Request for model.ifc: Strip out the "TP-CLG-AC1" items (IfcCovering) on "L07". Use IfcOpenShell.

First a look at what the model holds.

```python
import ifcopenshell
import ifcopenshell.util.element

model = ifcopenshell.open("model.ifc")
print(model.schema)
storey = next(s for s in model.by_type("IfcBuildingStorey") if s.Name == "L07")
coverings = [e for e in ifcopenshell.util.element.get_decomposition(storey) if e.is_a("IfcCovering")]
seen = {}
for e in coverings:
    element_type = ifcopenshell.util.element.get_type(e)
    name = element_type.Name if element_type not in (None, e) else None
    seen[name] = seen.get(name, 0) + 1
for name, count in sorted(seen.items(), key=str):
    print(count, "x", name)
```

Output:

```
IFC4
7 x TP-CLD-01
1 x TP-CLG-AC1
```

```python
import ifcopenshell
import ifcopenshell.api.root
import ifcopenshell.util.element

model = ifcopenshell.open("model.ifc")

storey = next(s for s in model.by_type("IfcBuildingStorey") if s.Name == "L07")
coverings = [e for e in ifcopenshell.util.element.get_decomposition(storey) if e.is_a("IfcCovering")]
targets = [e for e in coverings if (t := ifcopenshell.util.element.get_type(e)) not in (None, e) and t.Name == "TP-CLG-AC1"]

for e in targets:
    ifcopenshell.api.root.remove_product(model, product=e)
print(len(targets), "removed")

model.write("model-out.ifc")
```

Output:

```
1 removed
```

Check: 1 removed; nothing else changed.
